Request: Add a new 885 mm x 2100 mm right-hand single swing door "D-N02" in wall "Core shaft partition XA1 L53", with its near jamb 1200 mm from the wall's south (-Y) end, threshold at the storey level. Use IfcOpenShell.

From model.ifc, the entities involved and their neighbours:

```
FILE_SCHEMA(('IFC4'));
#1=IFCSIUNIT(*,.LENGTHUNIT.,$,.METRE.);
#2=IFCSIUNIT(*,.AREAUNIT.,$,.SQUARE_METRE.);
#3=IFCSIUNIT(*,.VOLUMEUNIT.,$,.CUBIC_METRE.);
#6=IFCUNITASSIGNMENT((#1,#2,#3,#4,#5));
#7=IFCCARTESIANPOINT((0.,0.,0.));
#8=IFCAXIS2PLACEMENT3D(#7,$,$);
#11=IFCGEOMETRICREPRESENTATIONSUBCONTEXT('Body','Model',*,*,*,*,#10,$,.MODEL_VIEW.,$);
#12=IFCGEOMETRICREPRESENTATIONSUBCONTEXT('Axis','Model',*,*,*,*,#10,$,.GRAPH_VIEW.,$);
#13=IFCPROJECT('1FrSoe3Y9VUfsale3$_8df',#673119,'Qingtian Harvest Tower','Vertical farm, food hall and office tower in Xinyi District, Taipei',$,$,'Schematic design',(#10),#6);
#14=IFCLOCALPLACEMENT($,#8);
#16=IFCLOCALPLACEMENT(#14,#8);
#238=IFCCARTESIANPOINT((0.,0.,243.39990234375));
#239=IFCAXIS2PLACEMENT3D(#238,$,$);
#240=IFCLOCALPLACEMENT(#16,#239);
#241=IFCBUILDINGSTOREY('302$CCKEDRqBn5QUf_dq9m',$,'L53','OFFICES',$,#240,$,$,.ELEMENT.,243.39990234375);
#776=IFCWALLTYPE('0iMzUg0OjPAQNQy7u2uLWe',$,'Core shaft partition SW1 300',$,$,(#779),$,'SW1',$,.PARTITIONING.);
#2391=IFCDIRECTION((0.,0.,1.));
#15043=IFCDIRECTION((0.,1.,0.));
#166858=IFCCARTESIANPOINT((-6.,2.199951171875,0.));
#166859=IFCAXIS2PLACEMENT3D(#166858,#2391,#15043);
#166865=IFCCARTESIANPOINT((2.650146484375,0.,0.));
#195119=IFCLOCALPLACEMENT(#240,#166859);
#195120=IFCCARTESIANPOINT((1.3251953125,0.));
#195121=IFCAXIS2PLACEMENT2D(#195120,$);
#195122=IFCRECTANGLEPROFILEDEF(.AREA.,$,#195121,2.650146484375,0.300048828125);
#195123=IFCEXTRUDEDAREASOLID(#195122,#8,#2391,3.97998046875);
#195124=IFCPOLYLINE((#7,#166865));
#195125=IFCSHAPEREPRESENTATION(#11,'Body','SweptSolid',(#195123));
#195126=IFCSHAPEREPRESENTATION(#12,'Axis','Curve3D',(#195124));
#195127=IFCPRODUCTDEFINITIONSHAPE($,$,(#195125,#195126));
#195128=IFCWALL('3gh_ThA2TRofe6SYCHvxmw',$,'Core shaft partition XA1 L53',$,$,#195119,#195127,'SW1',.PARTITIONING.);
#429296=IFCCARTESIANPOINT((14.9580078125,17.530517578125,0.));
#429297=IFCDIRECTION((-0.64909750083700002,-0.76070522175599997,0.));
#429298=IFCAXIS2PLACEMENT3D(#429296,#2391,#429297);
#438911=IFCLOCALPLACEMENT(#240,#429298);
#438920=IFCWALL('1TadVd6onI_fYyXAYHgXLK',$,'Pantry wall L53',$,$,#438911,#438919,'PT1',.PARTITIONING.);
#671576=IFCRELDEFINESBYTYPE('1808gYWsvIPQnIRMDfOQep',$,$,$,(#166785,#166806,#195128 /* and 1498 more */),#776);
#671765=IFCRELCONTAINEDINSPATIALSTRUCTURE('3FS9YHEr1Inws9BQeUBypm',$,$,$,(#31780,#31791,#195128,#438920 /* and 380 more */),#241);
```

```python
import numpy as np
import ifcopenshell
import ifcopenshell.api.feature
import ifcopenshell.api.geometry
import ifcopenshell.api.root
import ifcopenshell.api.spatial
import ifcopenshell.geom
import ifcopenshell.util.element
import ifcopenshell.util.placement
import ifcopenshell.util.representation
import ifcopenshell.util.shape
import ifcopenshell.util.unit

model = ifcopenshell.open("model.ifc")
unit_scale = ifcopenshell.util.unit.calculate_unit_scale(model)
settings = ifcopenshell.geom.settings()


def volume(element):
    """Net volume in cubic metres, openings subtracted."""
    shape = ifcopenshell.geom.create_shape(settings, element)
    return ifcopenshell.util.shape.get_volume(shape.geometry)


wall = model.by_guid("3gh_ThA2TRofe6SYCHvxmw")
storey = ifcopenshell.util.element.get_container(wall, ifc_class="IfcBuildingStorey")
context = ifcopenshell.util.representation.get_context(model, "Model", "Body", "MODEL_VIEW")
before = volume(wall)

width, height, from_end, sill = 0.885, 2.1, 1.2, 0.0  # metres

# The wall runs along its own X axis, and the end named is its -X end.
wall_shape = ifcopenshell.geom.create_shape(settings, wall)
x, y, z = ifcopenshell.util.shape.get_vertices(wall_shape.geometry).T
start = x.min() + from_end
face, thickness = float(y.min()), float(y.max() - y.min())
wall_matrix = ifcopenshell.util.placement.get_local_placement(wall.ObjectPlacement)
level = ifcopenshell.util.placement.get_local_placement(storey.ObjectPlacement)[2, 3]


def in_wall(x, y):
    """Placement at x, y metres in the wall's axes, at sill height."""
    matrix = wall_matrix.copy()
    matrix[:, 3] = wall_matrix @ np.array([x / unit_scale, y / unit_scale, 0.0, 1.0])
    matrix[2, 3] = level + sill / unit_scale
    return matrix


# Opening: a box that overshoots both wall faces by 50 mm.
opening = ifcopenshell.api.root.create_entity(model, ifc_class="IfcOpeningElement", predefined_type="OPENING")
box = ifcopenshell.api.geometry.add_wall_representation(
    model, context=context, length=width, height=height, thickness=thickness + 0.1
)
ifcopenshell.api.geometry.assign_representation(model, product=opening, representation=box)
ifcopenshell.api.geometry.edit_object_placement(model, product=opening, matrix=in_wall(start, face - 0.05), is_si=False)
ifcopenshell.api.feature.add_feature(model, feature=opening, element=wall)

door = ifcopenshell.api.root.create_entity(model, ifc_class="IfcDoor", name="D-N02", predefined_type="DOOR")
door.OverallWidth, door.OverallHeight = width / unit_scale, height / unit_scale
door.OperationType = "SINGLE_SWING_RIGHT"
body = ifcopenshell.api.geometry.add_door_representation(
    model,
    context=context,
    overall_width=door.OverallWidth,
    overall_height=door.OverallHeight,
    operation_type="SINGLE_SWING_RIGHT",
    lining_properties={"LiningDepth": thickness / unit_scale, "ThresholdDepth": thickness / unit_scale},
)
ifcopenshell.api.geometry.assign_representation(model, product=door, representation=body)
ifcopenshell.api.spatial.assign_container(model, products=[door], relating_structure=storey)
ifcopenshell.api.feature.add_filling(model, opening=opening, element=door)

# The lining spans the wall, so the door starts at the wall face.
ifcopenshell.api.geometry.edit_object_placement(model, product=door, matrix=in_wall(start, face), is_si=False)

after = volume(wall)

print(f"wall volume {before:.3f} -> {after:.3f} m3")

model.write("model-out.ifc")
```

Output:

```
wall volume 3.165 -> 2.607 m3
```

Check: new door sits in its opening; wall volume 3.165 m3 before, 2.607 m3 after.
